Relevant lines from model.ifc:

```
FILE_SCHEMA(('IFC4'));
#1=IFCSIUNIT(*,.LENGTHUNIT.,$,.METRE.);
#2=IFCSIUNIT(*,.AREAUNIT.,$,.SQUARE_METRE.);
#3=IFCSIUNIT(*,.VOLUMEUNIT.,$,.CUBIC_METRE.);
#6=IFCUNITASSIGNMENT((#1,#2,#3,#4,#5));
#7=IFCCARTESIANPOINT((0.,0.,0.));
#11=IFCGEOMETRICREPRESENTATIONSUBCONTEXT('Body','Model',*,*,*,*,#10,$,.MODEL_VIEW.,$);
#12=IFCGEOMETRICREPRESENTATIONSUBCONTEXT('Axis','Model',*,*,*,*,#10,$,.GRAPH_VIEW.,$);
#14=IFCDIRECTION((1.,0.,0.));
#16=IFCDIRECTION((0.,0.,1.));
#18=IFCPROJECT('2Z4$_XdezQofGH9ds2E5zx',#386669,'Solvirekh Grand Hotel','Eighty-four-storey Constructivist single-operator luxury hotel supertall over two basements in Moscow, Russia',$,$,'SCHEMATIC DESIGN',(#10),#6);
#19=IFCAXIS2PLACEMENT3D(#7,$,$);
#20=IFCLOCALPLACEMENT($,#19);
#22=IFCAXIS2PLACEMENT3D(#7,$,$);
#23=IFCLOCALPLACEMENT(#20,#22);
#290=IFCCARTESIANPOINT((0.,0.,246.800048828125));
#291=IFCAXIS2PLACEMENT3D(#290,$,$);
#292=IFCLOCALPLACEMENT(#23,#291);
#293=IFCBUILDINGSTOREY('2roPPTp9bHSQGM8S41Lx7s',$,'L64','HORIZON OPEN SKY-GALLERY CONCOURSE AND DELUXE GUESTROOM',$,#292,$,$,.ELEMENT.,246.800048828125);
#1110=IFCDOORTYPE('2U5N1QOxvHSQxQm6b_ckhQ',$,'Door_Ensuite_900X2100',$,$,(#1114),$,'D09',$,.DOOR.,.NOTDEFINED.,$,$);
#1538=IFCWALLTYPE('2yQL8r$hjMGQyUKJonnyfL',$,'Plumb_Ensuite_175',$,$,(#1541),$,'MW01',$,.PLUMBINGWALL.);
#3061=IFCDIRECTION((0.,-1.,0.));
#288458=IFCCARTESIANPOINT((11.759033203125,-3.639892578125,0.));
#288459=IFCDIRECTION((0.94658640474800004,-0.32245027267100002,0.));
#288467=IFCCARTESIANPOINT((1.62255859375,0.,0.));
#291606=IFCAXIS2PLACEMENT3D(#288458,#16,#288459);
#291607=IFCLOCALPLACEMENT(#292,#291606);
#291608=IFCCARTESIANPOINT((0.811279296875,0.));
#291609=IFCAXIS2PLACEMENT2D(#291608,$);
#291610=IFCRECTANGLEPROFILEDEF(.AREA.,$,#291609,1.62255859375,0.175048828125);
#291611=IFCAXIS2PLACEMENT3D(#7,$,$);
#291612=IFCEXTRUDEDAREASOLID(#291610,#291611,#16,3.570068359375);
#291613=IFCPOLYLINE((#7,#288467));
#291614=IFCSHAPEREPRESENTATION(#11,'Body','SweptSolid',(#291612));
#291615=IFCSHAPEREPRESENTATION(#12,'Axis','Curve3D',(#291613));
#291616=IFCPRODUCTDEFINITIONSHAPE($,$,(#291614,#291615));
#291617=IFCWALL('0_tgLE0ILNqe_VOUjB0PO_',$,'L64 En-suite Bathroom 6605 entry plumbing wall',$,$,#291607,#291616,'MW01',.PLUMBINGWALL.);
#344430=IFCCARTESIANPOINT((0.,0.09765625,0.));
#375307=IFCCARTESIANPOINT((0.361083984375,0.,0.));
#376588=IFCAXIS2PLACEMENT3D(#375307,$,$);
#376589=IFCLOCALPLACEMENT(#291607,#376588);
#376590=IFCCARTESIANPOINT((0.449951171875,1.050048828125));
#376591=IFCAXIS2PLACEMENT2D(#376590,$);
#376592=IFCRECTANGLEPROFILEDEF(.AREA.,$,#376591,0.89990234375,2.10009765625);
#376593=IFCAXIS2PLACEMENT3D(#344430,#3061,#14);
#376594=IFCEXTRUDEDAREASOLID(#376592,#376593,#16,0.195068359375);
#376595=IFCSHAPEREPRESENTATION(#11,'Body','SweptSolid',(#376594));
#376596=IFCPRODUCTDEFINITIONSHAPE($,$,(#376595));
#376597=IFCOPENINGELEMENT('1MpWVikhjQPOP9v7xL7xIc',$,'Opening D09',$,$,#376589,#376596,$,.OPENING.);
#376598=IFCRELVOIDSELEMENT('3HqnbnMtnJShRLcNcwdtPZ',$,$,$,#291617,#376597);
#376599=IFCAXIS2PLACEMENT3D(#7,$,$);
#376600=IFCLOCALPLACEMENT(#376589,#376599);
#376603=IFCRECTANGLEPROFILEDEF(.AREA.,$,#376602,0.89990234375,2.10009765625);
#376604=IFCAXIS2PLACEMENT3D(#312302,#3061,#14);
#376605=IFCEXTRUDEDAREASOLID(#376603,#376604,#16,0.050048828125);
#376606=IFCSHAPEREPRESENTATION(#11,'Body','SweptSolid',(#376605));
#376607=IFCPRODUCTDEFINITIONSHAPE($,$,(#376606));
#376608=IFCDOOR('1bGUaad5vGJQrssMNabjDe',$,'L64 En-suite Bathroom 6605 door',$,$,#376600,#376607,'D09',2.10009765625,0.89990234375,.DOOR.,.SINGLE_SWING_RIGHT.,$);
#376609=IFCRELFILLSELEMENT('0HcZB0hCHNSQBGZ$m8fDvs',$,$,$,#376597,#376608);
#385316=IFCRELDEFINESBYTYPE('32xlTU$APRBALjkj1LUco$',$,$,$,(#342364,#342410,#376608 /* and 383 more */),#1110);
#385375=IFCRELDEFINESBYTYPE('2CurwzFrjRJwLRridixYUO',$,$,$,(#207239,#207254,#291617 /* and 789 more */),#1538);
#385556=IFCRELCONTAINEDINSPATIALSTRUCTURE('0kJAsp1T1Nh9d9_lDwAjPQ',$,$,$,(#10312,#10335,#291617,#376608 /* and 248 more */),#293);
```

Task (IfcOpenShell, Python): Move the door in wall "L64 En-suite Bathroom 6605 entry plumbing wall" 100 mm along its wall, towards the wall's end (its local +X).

```python
import ifcopenshell
import ifcopenshell.api.geometry
import ifcopenshell.util.placement

model = ifcopenshell.open("model.ifc")

door = model.by_id(376608)
opening = door.FillsVoids[0].RelatingOpeningElement
wall = opening.VoidsElements[0].RelatingBuildingElement

wall_matrix = ifcopenshell.util.placement.get_local_placement(wall.ObjectPlacement)
shift = wall_matrix[:3, 0] * 0.1
before = ifcopenshell.util.placement.get_local_placement(door.ObjectPlacement)[:3, 3].copy()

# The door is placed relative to its opening, so it follows when the opening moves.
matrix = ifcopenshell.util.placement.get_local_placement(opening.ObjectPlacement)
matrix[:3, 3] += shift
ifcopenshell.api.geometry.edit_object_placement(
    model, product=opening, matrix=matrix, is_si=False, should_transform_children=True
)

after = ifcopenshell.util.placement.get_local_placement(door.ObjectPlacement)[:3, 3]
print("door moved by", (after - before).round(3) + 0.0)

model.write("model_v2.ifc")
```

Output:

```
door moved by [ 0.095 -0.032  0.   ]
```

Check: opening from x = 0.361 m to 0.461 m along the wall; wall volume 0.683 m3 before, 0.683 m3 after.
